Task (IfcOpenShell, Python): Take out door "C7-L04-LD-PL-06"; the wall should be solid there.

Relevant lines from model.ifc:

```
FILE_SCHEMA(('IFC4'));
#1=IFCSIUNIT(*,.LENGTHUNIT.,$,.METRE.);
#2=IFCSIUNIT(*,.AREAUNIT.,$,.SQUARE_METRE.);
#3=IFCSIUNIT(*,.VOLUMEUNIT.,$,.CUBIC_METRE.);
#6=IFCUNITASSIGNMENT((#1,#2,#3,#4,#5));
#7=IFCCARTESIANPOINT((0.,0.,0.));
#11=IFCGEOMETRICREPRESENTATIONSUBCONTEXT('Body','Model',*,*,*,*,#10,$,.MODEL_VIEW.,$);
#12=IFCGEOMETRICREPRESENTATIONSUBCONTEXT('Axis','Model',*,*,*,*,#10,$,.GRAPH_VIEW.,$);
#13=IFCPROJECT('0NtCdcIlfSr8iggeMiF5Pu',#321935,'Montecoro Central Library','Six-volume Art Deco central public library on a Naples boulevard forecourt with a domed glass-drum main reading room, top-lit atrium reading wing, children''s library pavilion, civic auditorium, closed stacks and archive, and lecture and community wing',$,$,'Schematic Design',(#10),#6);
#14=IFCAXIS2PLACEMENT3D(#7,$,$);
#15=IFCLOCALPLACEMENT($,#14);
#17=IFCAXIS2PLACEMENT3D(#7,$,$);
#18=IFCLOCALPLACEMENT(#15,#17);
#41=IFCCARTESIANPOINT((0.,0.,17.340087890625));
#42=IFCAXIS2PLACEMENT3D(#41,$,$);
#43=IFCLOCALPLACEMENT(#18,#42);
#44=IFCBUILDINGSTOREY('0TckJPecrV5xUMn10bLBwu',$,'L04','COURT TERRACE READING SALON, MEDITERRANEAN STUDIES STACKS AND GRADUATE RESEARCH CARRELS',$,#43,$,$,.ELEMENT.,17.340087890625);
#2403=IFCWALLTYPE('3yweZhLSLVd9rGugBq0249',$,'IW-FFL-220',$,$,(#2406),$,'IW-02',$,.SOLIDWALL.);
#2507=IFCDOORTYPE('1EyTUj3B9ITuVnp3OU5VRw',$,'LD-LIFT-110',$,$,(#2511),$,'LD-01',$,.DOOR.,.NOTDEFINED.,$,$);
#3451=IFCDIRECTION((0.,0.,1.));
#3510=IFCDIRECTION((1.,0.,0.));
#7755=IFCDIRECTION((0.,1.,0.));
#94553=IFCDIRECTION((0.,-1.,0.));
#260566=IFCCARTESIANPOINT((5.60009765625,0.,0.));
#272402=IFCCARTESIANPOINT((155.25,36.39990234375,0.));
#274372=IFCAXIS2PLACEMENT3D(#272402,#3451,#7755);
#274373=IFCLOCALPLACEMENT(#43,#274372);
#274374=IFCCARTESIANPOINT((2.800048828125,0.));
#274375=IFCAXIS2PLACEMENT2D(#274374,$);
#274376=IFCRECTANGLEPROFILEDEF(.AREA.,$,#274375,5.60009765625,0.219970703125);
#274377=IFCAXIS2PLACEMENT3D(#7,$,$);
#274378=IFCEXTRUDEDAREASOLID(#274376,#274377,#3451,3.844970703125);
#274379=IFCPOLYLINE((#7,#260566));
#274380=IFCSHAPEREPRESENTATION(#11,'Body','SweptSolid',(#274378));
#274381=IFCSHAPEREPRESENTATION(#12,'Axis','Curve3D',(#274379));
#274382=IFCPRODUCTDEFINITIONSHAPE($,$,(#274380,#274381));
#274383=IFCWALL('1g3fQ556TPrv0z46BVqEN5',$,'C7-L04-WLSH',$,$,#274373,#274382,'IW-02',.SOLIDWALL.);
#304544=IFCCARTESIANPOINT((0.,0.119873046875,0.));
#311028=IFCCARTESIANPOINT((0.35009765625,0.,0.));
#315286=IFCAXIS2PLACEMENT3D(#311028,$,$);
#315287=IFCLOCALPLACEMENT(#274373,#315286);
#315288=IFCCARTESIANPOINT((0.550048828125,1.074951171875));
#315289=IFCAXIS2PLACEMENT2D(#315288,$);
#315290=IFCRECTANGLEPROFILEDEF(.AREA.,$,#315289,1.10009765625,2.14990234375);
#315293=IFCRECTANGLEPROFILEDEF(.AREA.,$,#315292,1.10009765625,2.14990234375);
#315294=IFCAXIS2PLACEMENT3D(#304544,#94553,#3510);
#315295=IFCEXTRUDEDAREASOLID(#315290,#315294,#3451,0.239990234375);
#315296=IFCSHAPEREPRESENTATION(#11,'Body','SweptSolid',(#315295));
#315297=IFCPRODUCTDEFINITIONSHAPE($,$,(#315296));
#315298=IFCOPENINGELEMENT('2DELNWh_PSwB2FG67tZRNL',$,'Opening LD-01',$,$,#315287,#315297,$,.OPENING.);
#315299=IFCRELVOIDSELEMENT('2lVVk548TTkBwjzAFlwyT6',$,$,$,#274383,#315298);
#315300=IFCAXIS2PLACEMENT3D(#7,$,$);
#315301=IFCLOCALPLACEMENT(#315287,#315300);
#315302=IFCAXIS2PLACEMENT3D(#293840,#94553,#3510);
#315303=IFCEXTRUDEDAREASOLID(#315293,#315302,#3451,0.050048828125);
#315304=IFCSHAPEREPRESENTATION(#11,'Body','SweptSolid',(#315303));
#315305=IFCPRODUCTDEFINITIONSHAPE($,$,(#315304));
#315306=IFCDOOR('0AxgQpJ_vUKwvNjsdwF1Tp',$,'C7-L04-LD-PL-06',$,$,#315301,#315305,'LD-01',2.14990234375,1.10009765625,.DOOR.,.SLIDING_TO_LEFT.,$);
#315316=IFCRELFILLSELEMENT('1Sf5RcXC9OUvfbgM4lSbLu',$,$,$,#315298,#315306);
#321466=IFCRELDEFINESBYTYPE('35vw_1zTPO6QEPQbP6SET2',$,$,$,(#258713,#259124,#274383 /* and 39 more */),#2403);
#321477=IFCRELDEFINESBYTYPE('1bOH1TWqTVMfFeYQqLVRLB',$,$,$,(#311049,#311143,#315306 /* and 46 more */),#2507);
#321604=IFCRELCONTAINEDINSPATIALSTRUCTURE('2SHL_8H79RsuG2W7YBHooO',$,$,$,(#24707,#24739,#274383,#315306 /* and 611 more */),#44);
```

```python
import ifcopenshell
import ifcopenshell.api.feature
import ifcopenshell.api.root
import ifcopenshell.geom
import ifcopenshell.util.shape

model = ifcopenshell.open("model.ifc")
settings = ifcopenshell.geom.settings()


def volume(element):
    """Net volume in cubic metres, openings subtracted."""
    shape = ifcopenshell.geom.create_shape(settings, element)
    return ifcopenshell.util.shape.get_volume(shape.geometry)


door = model.by_id(315306)
opening = door.FillsVoids[0].RelatingOpeningElement
wall = opening.VoidsElements[0].RelatingBuildingElement
before = volume(wall)

ifcopenshell.api.root.remove_product(model, product=door)
ifcopenshell.api.feature.remove_feature(model, feature=opening)

after = volume(wall)

print(f"wall volume {before:.3f} -> {after:.3f} m3")

model.write("model_updated.ifc")
```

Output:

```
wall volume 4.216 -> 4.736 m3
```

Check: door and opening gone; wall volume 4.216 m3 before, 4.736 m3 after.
